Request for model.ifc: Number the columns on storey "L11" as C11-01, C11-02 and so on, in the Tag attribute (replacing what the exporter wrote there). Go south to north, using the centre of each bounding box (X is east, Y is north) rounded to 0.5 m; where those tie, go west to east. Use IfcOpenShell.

First a look at what the model holds.

```python
import ifcopenshell
import ifcopenshell.util.element
import ifcopenshell.util.placement

model = ifcopenshell.open("model.ifc")
print(model.schema)
storey = next(s for s in model.by_type("IfcBuildingStorey") if s.Name == "L11")
columns = [e for e in ifcopenshell.util.element.get_decomposition(storey) if e.is_a("IfcColumn")]
for e in sorted(columns, key=lambda e: e.id()):
    origin = ifcopenshell.util.placement.get_local_placement(e.ObjectPlacement)[:3, 3]
    print(e.id(), e.Tag, e.Name, origin.round(2) + 0.0, sep=" | ")
```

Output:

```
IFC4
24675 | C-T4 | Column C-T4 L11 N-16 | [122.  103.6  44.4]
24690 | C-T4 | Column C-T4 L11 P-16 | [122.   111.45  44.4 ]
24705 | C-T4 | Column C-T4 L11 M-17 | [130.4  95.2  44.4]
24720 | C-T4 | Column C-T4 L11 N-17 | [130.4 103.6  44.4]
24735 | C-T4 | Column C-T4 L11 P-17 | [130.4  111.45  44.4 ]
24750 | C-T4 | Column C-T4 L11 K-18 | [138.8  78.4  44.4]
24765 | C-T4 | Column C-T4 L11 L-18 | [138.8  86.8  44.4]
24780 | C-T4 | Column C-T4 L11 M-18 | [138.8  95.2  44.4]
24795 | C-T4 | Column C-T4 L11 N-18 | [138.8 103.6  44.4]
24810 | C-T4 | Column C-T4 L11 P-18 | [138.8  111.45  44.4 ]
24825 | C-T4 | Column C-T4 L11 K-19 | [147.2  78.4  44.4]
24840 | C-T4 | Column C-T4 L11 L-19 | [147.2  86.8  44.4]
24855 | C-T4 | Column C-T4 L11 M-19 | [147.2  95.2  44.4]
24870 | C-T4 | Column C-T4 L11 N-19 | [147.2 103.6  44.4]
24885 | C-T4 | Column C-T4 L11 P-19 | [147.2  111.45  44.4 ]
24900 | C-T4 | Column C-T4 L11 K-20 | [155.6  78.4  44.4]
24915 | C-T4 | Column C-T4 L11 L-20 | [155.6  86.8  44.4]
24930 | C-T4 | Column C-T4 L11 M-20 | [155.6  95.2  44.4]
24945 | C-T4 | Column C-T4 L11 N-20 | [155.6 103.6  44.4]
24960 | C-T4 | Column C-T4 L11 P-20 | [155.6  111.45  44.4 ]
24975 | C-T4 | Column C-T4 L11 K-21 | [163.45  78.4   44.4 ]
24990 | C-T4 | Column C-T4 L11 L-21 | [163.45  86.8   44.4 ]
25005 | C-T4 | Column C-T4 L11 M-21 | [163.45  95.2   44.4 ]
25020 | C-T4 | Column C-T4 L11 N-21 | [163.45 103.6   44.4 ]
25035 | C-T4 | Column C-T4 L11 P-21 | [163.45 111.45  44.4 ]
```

```python
import ifcopenshell
import ifcopenshell.geom
import ifcopenshell.util.element
import ifcopenshell.util.shape

model = ifcopenshell.open("model.ifc")
settings = ifcopenshell.geom.settings()
settings.set("use-world-coords", True)


def centre(element):
    shape = ifcopenshell.geom.create_shape(settings, element)
    return ifcopenshell.util.shape.get_bbox_centroid(shape.geometry)


storey = next(s for s in model.by_type("IfcBuildingStorey") if s.Name == "L11")
columns = [e for e in ifcopenshell.util.element.get_decomposition(storey) if e.is_a("IfcColumn")]

# Insertion points can sit at a corner or the storey origin, so sort by the geometry (in metres).
centres = {e: centre(e) for e in columns}
columns.sort(key=lambda e: (round(centres[e][1] / 0.5), centres[e][0]))

for i, e in enumerate(columns, start=1):
    number = f"C11-{i:02d}"
    e.Tag = number
    print(e.id(), number)

model.write("model_edited.ifc")
```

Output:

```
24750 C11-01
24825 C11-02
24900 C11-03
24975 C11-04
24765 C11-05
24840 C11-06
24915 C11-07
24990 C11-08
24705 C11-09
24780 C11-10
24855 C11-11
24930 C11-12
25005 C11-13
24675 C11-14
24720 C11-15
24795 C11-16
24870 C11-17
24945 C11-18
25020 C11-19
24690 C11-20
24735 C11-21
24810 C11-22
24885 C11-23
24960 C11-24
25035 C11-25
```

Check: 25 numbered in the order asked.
